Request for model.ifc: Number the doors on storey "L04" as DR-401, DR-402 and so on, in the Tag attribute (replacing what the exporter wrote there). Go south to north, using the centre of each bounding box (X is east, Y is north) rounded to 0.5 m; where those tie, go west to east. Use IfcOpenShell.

First a look at what the model holds.

```python
import ifcopenshell
import ifcopenshell.util.element
import ifcopenshell.util.placement

model = ifcopenshell.open("model.ifc")
print(model.schema)
storey = next(s for s in model.by_type("IfcBuildingStorey") if s.Name == "L04")
doors = [e for e in ifcopenshell.util.element.get_decomposition(storey) if e.is_a("IfcDoor")]
for e in sorted(doors, key=lambda e: e.id()):
    origin = ifcopenshell.util.placement.get_local_placement(e.ObjectPlacement)[:3, 3]
    print(e.id(), e.Tag, e.Name, origin.round(2) + 0.0, sep=" | ")
```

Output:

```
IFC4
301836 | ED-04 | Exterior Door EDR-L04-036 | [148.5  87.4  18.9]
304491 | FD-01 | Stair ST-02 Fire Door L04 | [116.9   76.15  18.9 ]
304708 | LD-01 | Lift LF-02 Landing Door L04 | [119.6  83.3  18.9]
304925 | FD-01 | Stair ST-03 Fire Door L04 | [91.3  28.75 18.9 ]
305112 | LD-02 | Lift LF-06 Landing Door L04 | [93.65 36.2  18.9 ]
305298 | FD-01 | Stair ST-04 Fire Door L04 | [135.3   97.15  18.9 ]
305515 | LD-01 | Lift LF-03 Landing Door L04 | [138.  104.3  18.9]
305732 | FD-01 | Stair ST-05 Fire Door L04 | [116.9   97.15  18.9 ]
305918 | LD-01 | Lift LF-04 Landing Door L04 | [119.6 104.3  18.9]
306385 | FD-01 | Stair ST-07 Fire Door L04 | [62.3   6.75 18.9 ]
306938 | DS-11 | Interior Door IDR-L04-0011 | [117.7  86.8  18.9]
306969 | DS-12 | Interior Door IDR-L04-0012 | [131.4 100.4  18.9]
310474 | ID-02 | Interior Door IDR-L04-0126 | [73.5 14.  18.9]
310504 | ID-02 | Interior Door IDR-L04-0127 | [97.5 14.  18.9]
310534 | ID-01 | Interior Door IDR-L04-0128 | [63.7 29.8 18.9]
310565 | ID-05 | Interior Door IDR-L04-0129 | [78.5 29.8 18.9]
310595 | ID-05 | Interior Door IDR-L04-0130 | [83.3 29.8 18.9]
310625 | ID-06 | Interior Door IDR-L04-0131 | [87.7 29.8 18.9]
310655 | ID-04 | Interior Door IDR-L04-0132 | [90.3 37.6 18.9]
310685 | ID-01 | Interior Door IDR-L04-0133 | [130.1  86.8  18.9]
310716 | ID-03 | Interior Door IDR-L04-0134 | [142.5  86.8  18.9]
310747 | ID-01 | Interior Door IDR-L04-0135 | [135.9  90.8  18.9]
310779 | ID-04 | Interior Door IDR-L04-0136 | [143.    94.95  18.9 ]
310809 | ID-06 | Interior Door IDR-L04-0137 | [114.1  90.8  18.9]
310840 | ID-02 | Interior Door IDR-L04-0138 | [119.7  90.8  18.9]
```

```python
import ifcopenshell
import ifcopenshell.geom
import ifcopenshell.util.element
import ifcopenshell.util.shape

model = ifcopenshell.open("model.ifc")
settings = ifcopenshell.geom.settings()
settings.set("use-world-coords", True)


def centre(element):
    shape = ifcopenshell.geom.create_shape(settings, element)
    return ifcopenshell.util.shape.get_bbox_centroid(shape.geometry)


storey = next(s for s in model.by_type("IfcBuildingStorey") if s.Name == "L04")
doors = [e for e in ifcopenshell.util.element.get_decomposition(storey) if e.is_a("IfcDoor")]

# Insertion points can sit at a corner or the storey origin, so sort by the geometry (in metres).
centres = {e: centre(e) for e in doors}
doors.sort(key=lambda e: (round(centres[e][1] / 0.5), centres[e][0]))

for i, e in enumerate(doors, start=1):
    number = f"DR-4{i:02d}"
    e.Tag = number
    print(e.id(), number)

model.write("model-out.ifc")
```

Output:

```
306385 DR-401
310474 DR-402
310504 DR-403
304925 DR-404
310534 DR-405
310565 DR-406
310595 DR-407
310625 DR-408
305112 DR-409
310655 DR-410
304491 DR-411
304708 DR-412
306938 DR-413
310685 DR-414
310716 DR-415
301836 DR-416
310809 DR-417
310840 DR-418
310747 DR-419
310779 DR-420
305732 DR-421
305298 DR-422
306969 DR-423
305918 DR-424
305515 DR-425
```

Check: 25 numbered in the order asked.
